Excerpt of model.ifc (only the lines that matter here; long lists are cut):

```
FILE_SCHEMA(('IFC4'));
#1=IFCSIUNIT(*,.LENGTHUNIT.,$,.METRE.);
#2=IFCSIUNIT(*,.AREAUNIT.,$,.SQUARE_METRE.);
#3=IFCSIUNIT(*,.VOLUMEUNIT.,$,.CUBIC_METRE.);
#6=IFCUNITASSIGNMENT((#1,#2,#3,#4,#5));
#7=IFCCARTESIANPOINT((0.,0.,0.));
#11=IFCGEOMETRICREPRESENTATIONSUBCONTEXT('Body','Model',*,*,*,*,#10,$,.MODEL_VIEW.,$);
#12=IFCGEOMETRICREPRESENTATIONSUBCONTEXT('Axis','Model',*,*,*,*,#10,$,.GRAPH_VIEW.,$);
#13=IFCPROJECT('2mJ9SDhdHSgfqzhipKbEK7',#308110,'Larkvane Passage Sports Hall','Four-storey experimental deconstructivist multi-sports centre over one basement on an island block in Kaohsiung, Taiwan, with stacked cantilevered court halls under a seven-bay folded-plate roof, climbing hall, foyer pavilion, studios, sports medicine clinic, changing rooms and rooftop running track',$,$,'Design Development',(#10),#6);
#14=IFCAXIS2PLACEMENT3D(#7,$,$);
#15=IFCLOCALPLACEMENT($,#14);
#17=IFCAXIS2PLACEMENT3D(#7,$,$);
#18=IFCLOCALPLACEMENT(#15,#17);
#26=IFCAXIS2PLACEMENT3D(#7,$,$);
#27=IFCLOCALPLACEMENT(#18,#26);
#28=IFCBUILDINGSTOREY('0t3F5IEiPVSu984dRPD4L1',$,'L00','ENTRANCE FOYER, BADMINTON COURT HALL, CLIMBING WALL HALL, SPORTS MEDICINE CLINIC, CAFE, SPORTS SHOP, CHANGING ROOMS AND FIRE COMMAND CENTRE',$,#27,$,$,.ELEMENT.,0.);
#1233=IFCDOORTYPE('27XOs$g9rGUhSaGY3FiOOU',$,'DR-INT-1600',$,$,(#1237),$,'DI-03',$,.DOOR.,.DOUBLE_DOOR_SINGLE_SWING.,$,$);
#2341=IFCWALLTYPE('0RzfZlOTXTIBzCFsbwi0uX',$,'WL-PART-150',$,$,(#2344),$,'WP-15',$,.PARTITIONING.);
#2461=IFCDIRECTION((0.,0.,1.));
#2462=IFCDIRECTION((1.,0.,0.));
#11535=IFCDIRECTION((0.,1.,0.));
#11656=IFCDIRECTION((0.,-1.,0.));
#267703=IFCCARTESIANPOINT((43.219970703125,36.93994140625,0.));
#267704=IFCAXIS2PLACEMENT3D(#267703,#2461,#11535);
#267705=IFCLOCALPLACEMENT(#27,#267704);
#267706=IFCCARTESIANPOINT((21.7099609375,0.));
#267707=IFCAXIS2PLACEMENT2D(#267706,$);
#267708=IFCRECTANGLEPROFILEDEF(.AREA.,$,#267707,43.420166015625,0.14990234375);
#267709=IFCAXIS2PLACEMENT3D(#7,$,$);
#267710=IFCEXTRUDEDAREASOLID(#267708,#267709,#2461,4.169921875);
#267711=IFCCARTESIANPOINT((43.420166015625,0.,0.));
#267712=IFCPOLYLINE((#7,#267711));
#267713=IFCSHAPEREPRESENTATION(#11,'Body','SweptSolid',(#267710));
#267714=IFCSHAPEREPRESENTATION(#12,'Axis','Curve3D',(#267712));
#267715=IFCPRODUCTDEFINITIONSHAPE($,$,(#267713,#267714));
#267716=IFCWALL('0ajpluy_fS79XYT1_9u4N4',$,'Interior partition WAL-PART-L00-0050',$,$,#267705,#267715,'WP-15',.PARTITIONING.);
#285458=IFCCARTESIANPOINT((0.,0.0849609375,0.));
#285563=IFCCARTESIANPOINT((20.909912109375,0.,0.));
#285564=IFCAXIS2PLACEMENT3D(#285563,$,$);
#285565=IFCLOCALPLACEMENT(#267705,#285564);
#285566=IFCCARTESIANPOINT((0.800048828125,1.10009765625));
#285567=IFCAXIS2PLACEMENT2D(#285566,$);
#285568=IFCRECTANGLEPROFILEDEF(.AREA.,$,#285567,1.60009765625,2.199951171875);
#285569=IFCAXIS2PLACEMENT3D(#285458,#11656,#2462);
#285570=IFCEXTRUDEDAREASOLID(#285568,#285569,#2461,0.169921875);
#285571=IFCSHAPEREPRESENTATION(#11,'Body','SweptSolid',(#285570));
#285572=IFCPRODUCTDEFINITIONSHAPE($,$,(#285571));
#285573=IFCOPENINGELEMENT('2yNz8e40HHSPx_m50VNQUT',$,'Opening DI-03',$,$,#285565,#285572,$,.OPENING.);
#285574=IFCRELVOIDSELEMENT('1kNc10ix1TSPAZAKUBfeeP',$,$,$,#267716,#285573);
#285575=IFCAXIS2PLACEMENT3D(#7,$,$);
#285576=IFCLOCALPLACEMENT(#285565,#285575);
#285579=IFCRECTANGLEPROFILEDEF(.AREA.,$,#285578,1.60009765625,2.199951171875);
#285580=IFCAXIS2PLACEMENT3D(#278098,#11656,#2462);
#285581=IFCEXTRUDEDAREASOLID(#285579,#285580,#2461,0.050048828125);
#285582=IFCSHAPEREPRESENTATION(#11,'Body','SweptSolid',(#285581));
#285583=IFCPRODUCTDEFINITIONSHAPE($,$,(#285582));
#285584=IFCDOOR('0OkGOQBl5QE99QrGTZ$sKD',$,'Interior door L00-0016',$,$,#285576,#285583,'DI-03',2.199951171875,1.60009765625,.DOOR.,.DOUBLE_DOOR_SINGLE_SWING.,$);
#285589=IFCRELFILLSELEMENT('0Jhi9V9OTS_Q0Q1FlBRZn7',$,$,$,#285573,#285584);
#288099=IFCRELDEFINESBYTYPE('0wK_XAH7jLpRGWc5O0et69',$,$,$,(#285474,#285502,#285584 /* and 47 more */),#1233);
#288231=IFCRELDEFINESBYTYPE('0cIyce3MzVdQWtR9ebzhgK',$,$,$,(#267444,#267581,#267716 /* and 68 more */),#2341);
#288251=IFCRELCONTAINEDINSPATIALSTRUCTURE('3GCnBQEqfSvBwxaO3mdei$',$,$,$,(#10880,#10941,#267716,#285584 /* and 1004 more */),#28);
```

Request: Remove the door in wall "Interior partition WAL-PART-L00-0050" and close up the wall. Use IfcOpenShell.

```python
import ifcopenshell
import ifcopenshell.api.feature
import ifcopenshell.api.root
import ifcopenshell.geom
import ifcopenshell.util.shape

model = ifcopenshell.open("model.ifc")
settings = ifcopenshell.geom.settings()


def volume(element):
    """Net volume in cubic metres, openings subtracted."""
    shape = ifcopenshell.geom.create_shape(settings, element)
    return ifcopenshell.util.shape.get_volume(shape.geometry)


door = model.by_id(285584)
opening = door.FillsVoids[0].RelatingOpeningElement
wall = opening.VoidsElements[0].RelatingBuildingElement
before = volume(wall)

ifcopenshell.api.root.remove_product(model, product=door)
ifcopenshell.api.feature.remove_feature(model, feature=opening)

after = volume(wall)

print(f"wall volume {before:.3f} -> {after:.3f} m3")

model.write("model_updated.ifc")
```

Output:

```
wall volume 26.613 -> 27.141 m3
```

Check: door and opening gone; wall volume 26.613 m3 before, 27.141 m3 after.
